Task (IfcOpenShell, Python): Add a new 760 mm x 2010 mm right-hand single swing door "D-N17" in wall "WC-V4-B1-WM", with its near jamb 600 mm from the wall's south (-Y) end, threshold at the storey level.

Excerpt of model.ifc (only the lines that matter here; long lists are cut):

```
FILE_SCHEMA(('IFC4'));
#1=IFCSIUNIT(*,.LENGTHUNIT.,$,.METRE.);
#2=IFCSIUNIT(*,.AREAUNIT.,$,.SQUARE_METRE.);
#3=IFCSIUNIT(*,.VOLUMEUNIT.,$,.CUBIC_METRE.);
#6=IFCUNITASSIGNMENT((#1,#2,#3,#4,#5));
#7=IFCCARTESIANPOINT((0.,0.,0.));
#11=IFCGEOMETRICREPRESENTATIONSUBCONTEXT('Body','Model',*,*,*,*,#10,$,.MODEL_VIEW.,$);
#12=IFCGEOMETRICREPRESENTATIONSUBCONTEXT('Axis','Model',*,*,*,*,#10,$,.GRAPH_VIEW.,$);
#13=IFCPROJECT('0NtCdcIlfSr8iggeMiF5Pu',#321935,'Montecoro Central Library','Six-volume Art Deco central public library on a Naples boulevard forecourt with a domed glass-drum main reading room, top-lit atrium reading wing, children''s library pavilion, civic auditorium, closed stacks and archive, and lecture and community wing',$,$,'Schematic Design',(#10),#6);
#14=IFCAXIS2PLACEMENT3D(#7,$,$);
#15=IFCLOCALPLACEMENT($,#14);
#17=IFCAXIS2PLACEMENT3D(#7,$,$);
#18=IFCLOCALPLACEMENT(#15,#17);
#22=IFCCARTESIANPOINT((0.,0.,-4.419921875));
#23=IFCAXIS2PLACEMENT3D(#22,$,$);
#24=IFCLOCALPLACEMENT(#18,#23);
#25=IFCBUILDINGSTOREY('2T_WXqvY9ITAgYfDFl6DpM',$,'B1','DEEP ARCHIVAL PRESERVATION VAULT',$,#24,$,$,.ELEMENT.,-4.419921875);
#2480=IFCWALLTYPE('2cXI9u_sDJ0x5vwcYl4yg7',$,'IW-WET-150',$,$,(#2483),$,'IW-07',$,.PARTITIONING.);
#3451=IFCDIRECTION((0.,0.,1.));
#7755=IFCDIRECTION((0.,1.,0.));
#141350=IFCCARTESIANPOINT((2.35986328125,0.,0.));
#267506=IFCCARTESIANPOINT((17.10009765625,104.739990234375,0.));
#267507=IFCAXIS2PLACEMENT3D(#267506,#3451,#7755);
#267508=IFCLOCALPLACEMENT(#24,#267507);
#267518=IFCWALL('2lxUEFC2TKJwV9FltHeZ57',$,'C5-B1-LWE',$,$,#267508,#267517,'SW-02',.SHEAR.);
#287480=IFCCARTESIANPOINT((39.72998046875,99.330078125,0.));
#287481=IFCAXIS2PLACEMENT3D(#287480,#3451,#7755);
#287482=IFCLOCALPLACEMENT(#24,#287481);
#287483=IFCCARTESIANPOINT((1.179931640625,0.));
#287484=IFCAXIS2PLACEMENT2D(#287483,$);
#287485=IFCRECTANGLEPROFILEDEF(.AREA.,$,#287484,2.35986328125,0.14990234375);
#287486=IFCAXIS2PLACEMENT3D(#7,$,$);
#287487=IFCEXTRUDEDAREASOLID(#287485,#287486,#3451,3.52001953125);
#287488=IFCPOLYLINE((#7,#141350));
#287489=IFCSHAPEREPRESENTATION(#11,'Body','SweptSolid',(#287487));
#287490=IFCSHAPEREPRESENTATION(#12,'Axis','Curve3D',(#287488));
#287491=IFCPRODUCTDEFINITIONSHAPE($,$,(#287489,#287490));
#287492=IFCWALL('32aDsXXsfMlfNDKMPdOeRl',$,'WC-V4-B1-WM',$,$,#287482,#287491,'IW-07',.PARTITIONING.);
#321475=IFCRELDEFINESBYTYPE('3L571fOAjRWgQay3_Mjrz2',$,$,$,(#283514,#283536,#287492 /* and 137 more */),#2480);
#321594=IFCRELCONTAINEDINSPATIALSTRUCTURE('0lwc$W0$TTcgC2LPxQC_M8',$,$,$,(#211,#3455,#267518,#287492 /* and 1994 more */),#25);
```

```python
import numpy as np
import ifcopenshell
import ifcopenshell.api.feature
import ifcopenshell.api.geometry
import ifcopenshell.api.root
import ifcopenshell.api.spatial
import ifcopenshell.geom
import ifcopenshell.util.element
import ifcopenshell.util.placement
import ifcopenshell.util.representation
import ifcopenshell.util.shape
import ifcopenshell.util.unit

model = ifcopenshell.open("model.ifc")
unit_scale = ifcopenshell.util.unit.calculate_unit_scale(model)
settings = ifcopenshell.geom.settings()


def volume(element):
    """Net volume in cubic metres, openings subtracted."""
    shape = ifcopenshell.geom.create_shape(settings, element)
    return ifcopenshell.util.shape.get_volume(shape.geometry)


wall = model.by_guid("32aDsXXsfMlfNDKMPdOeRl")
storey = ifcopenshell.util.element.get_container(wall, ifc_class="IfcBuildingStorey")
context = ifcopenshell.util.representation.get_context(model, "Model", "Body", "MODEL_VIEW")
before = volume(wall)

width, height, from_end, sill = 0.76, 2.01, 0.6, 0.0  # metres

# The wall runs along its own X axis, and the end named is its -X end.
wall_shape = ifcopenshell.geom.create_shape(settings, wall)
x, y, z = ifcopenshell.util.shape.get_vertices(wall_shape.geometry).T
start = x.min() + from_end
face, thickness = float(y.min()), float(y.max() - y.min())
wall_matrix = ifcopenshell.util.placement.get_local_placement(wall.ObjectPlacement)
level = ifcopenshell.util.placement.get_local_placement(storey.ObjectPlacement)[2, 3]


def in_wall(x, y):
    """Placement at x, y metres in the wall's axes, at sill height."""
    matrix = wall_matrix.copy()
    matrix[:, 3] = wall_matrix @ np.array([x / unit_scale, y / unit_scale, 0.0, 1.0])
    matrix[2, 3] = level + sill / unit_scale
    return matrix


# Opening: a box that overshoots both wall faces by 50 mm.
opening = ifcopenshell.api.root.create_entity(model, ifc_class="IfcOpeningElement", predefined_type="OPENING")
box = ifcopenshell.api.geometry.add_wall_representation(
    model, context=context, length=width, height=height, thickness=thickness + 0.1
)
ifcopenshell.api.geometry.assign_representation(model, product=opening, representation=box)
ifcopenshell.api.geometry.edit_object_placement(model, product=opening, matrix=in_wall(start, face - 0.05), is_si=False)
ifcopenshell.api.feature.add_feature(model, feature=opening, element=wall)

door = ifcopenshell.api.root.create_entity(model, ifc_class="IfcDoor", name="D-N17", predefined_type="DOOR")
door.OverallWidth, door.OverallHeight = width / unit_scale, height / unit_scale
door.OperationType = "SINGLE_SWING_RIGHT"
body = ifcopenshell.api.geometry.add_door_representation(
    model,
    context=context,
    overall_width=door.OverallWidth,
    overall_height=door.OverallHeight,
    operation_type="SINGLE_SWING_RIGHT",
    lining_properties={"LiningDepth": thickness / unit_scale, "ThresholdDepth": thickness / unit_scale},
)
ifcopenshell.api.geometry.assign_representation(model, product=door, representation=body)
ifcopenshell.api.spatial.assign_container(model, products=[door], relating_structure=storey)
ifcopenshell.api.feature.add_filling(model, opening=opening, element=door)

# The lining spans the wall, so the door starts at the wall face.
ifcopenshell.api.geometry.edit_object_placement(model, product=door, matrix=in_wall(start, face), is_si=False)

after = volume(wall)

print(f"wall volume {before:.3f} -> {after:.3f} m3")

model.write("model_updated.ifc")
```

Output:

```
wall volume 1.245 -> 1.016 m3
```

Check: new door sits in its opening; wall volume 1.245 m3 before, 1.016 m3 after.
